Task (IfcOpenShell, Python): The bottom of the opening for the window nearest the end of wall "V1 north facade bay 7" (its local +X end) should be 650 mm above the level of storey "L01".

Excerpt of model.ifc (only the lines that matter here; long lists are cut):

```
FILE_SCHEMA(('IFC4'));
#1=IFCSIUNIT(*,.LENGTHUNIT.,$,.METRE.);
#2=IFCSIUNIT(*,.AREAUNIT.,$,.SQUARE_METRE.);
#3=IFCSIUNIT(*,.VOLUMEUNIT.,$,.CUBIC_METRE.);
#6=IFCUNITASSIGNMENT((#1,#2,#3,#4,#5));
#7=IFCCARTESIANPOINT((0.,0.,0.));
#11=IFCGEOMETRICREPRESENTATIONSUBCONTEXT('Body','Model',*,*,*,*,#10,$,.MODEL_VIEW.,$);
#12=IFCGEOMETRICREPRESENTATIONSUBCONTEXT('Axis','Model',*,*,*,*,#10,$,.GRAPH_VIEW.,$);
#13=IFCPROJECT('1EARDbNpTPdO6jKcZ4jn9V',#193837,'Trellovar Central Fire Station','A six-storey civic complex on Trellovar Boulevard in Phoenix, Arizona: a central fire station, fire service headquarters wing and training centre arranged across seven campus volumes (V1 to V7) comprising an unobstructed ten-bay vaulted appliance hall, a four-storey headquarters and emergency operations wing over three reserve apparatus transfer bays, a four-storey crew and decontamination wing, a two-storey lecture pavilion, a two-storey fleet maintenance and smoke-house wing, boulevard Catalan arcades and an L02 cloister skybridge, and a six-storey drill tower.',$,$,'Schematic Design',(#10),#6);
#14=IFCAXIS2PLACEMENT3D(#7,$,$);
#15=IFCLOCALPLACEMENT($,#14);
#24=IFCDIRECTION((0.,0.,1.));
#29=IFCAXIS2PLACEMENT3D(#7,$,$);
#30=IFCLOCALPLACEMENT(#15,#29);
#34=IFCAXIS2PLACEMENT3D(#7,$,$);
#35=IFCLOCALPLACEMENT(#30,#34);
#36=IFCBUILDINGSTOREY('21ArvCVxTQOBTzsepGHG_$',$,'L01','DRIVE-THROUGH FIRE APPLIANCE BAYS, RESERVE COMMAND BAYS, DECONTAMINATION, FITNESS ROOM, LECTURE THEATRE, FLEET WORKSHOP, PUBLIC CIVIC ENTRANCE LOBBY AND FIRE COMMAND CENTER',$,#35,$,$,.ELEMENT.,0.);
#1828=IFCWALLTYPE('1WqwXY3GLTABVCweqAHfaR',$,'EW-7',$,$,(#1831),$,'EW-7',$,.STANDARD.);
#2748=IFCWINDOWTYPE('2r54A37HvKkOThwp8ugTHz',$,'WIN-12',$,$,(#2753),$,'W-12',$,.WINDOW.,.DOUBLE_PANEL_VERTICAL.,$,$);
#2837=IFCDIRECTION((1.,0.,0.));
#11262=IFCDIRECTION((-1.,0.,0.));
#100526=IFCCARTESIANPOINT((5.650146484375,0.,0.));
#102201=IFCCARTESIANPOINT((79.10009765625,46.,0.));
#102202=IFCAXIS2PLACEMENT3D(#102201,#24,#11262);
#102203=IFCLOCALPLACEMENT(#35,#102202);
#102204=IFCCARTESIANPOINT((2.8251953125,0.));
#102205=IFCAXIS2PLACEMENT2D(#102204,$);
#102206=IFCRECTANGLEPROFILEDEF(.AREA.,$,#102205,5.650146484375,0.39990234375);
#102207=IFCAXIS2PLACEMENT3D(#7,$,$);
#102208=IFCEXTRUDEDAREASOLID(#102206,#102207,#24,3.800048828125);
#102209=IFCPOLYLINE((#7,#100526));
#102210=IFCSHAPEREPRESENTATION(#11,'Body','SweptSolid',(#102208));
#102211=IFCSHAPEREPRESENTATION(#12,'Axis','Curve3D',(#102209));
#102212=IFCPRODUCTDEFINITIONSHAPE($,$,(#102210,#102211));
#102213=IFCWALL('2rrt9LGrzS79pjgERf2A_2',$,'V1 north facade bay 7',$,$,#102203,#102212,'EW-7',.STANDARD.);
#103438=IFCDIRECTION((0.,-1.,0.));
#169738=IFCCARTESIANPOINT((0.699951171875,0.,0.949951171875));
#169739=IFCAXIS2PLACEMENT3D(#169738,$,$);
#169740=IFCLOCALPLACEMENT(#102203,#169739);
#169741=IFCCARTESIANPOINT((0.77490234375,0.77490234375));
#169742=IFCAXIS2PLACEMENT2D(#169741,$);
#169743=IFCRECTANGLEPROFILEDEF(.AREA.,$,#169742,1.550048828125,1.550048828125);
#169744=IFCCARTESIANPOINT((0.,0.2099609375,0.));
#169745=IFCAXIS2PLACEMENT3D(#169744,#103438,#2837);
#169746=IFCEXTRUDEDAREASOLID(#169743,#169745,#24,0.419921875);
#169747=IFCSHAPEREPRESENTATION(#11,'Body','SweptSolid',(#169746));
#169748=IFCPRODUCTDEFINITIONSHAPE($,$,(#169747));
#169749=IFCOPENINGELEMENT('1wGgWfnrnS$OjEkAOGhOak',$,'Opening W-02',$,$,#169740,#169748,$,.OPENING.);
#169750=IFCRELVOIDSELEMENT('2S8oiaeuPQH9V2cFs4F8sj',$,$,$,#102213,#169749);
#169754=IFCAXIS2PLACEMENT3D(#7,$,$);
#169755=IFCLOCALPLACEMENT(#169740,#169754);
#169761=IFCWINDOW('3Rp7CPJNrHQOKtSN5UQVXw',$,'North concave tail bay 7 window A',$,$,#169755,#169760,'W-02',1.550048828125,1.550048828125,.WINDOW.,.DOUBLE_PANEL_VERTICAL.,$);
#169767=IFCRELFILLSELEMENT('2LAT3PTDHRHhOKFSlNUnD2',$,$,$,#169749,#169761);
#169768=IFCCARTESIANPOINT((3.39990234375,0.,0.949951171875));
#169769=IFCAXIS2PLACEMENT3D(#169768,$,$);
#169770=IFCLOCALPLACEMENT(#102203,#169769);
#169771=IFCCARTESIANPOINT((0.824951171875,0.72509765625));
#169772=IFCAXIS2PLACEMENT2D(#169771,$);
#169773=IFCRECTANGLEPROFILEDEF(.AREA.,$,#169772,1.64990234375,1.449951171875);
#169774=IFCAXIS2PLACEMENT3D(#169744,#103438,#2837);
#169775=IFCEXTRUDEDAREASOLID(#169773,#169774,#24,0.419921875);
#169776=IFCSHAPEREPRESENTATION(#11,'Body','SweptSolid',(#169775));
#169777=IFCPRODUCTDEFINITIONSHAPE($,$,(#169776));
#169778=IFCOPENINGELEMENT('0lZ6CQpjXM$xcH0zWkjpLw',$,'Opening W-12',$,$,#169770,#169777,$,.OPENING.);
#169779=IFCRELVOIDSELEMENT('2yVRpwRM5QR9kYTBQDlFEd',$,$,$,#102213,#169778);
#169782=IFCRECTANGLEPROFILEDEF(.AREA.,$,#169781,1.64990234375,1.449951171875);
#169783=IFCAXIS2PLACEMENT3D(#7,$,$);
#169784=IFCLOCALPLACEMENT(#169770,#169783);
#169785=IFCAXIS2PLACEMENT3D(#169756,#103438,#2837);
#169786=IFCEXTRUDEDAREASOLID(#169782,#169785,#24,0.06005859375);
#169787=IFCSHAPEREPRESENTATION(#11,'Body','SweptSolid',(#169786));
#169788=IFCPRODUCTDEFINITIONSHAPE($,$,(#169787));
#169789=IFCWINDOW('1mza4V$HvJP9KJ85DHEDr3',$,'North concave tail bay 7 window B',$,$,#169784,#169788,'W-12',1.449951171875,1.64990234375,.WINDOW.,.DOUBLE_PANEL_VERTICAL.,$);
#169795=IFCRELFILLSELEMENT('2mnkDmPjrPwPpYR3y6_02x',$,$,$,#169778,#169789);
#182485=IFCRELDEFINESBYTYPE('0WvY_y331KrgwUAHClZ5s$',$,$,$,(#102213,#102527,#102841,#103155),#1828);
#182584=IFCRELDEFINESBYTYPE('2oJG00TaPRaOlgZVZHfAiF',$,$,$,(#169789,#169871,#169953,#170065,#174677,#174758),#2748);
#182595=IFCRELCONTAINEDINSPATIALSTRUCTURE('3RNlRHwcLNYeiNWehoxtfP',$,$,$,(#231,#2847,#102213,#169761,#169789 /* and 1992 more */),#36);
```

```python
import numpy as np
import ifcopenshell
import ifcopenshell.api.geometry
import ifcopenshell.geom
import ifcopenshell.util.element
import ifcopenshell.util.placement
import ifcopenshell.util.shape
import ifcopenshell.util.unit

model = ifcopenshell.open("model.ifc")
unit_scale = ifcopenshell.util.unit.calculate_unit_scale(model)

window = model.by_guid("1mza4V$HvJP9KJ85DHEDr3")
opening = window.FillsVoids[0].RelatingOpeningElement
storey = ifcopenshell.util.element.get_container(window, ifc_class="IfcBuildingStorey")
level = ifcopenshell.util.placement.get_local_placement(storey.ObjectPlacement)[2, 3]

# The opening's origin need not be at the sill, so measure its lowest point.
shape = ifcopenshell.geom.create_shape(ifcopenshell.geom.settings(), opening)
bottom = ifcopenshell.util.shape.get_shape_bottom_elevation(shape, shape.geometry) / unit_scale
dz = level + 0.65 / unit_scale - bottom

shift = np.array([0.0, 0.0, dz])
# The window is placed relative to its opening, so it follows when the opening moves.
matrix = ifcopenshell.util.placement.get_local_placement(opening.ObjectPlacement)
matrix[:3, 3] += shift
ifcopenshell.api.geometry.edit_object_placement(
    model, product=opening, matrix=matrix, is_si=False, should_transform_children=True
)

print(f"moved by {dz * unit_scale:+.3f} m")

model.write("model_updated.ifc")
```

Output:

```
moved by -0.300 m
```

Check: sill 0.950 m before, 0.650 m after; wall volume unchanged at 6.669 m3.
